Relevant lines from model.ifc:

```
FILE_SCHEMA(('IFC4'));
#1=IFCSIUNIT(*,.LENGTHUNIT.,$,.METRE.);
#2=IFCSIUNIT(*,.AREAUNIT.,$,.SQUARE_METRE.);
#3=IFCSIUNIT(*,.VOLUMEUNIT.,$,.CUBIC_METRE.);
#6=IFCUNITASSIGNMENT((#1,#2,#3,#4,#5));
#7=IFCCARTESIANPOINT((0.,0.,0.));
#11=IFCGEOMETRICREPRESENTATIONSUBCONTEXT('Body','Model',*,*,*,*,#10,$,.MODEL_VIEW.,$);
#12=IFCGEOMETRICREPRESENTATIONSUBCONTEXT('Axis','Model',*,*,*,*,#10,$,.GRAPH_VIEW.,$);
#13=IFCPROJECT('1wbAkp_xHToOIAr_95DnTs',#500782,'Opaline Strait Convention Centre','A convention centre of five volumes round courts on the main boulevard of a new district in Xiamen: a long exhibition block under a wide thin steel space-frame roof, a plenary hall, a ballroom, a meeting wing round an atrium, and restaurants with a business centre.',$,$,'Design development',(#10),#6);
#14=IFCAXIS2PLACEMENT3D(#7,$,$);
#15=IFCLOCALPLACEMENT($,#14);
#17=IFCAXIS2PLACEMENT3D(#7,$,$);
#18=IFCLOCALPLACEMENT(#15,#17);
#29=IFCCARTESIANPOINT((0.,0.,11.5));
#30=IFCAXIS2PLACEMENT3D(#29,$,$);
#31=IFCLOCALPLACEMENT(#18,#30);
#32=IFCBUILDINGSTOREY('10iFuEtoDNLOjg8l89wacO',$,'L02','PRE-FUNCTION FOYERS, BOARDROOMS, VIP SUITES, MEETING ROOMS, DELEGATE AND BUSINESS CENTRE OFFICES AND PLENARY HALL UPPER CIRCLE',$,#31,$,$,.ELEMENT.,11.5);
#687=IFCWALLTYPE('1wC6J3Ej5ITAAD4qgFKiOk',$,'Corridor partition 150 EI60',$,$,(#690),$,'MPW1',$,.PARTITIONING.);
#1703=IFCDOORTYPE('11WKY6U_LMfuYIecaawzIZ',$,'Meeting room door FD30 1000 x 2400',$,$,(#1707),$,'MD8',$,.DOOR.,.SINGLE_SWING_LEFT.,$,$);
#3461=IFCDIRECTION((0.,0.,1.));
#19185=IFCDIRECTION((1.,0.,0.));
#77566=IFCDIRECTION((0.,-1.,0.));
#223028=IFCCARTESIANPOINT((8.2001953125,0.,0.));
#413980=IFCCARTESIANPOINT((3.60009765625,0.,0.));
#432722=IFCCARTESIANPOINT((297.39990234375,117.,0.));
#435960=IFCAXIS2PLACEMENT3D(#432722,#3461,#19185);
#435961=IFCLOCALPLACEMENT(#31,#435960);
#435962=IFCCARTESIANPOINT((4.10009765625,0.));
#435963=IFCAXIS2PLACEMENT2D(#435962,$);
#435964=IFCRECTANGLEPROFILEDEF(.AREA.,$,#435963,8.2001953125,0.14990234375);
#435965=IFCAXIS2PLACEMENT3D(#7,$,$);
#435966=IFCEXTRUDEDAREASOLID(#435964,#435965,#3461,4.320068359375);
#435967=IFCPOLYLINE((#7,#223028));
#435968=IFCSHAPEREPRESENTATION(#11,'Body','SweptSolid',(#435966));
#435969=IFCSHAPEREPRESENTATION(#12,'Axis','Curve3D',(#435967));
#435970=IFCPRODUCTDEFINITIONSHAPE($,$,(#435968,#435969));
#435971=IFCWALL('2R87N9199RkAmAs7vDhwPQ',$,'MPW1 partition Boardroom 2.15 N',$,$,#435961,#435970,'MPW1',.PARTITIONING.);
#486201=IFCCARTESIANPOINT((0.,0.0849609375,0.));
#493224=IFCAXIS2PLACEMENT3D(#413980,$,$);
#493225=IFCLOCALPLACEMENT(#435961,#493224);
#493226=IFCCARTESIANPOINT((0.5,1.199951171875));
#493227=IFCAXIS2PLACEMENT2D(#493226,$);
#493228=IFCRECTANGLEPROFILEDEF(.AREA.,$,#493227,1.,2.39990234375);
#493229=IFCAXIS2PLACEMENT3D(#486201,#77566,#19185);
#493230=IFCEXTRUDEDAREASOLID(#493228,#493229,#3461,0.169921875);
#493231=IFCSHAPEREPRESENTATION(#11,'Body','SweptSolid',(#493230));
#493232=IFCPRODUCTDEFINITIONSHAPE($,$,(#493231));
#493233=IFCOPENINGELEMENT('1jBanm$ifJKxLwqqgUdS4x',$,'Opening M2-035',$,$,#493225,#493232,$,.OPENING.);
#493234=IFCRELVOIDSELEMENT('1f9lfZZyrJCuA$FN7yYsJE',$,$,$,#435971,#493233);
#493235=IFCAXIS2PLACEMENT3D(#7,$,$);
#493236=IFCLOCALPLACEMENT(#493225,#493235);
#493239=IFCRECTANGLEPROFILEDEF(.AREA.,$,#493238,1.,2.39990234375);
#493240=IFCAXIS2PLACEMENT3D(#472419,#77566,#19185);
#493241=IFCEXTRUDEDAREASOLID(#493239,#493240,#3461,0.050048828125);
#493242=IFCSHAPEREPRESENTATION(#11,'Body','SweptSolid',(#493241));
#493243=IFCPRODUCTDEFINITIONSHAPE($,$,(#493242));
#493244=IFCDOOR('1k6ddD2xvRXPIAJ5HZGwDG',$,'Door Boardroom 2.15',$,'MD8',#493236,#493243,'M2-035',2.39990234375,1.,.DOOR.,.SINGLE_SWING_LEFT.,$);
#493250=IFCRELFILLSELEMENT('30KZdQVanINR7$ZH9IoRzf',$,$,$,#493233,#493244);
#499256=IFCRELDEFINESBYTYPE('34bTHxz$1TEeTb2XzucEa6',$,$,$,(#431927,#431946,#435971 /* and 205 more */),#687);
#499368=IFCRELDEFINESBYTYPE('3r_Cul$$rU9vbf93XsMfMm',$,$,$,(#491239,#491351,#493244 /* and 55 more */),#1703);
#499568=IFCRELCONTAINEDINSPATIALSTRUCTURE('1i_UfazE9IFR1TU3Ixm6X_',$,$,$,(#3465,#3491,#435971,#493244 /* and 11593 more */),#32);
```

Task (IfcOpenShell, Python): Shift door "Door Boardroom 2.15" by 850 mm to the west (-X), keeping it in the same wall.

```python
import ifcopenshell
import ifcopenshell.api.geometry
import ifcopenshell.util.placement

model = ifcopenshell.open("model.ifc")

door = model.by_id(493244)
opening = door.FillsVoids[0].RelatingOpeningElement
wall = opening.VoidsElements[0].RelatingBuildingElement

wall_matrix = ifcopenshell.util.placement.get_local_placement(wall.ObjectPlacement)
shift = wall_matrix[:3, 0] * -0.85
before = ifcopenshell.util.placement.get_local_placement(door.ObjectPlacement)[:3, 3].copy()

# The door is placed relative to its opening, so it follows when the opening moves.
matrix = ifcopenshell.util.placement.get_local_placement(opening.ObjectPlacement)
matrix[:3, 3] += shift
ifcopenshell.api.geometry.edit_object_placement(
    model, product=opening, matrix=matrix, is_si=False, should_transform_children=True
)

after = ifcopenshell.util.placement.get_local_placement(door.ObjectPlacement)[:3, 3]
print("door moved by", (after - before).round(3) + 0.0)

model.write("model_v2.ifc")
```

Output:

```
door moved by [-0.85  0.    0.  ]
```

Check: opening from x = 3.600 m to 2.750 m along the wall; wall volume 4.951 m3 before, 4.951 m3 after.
